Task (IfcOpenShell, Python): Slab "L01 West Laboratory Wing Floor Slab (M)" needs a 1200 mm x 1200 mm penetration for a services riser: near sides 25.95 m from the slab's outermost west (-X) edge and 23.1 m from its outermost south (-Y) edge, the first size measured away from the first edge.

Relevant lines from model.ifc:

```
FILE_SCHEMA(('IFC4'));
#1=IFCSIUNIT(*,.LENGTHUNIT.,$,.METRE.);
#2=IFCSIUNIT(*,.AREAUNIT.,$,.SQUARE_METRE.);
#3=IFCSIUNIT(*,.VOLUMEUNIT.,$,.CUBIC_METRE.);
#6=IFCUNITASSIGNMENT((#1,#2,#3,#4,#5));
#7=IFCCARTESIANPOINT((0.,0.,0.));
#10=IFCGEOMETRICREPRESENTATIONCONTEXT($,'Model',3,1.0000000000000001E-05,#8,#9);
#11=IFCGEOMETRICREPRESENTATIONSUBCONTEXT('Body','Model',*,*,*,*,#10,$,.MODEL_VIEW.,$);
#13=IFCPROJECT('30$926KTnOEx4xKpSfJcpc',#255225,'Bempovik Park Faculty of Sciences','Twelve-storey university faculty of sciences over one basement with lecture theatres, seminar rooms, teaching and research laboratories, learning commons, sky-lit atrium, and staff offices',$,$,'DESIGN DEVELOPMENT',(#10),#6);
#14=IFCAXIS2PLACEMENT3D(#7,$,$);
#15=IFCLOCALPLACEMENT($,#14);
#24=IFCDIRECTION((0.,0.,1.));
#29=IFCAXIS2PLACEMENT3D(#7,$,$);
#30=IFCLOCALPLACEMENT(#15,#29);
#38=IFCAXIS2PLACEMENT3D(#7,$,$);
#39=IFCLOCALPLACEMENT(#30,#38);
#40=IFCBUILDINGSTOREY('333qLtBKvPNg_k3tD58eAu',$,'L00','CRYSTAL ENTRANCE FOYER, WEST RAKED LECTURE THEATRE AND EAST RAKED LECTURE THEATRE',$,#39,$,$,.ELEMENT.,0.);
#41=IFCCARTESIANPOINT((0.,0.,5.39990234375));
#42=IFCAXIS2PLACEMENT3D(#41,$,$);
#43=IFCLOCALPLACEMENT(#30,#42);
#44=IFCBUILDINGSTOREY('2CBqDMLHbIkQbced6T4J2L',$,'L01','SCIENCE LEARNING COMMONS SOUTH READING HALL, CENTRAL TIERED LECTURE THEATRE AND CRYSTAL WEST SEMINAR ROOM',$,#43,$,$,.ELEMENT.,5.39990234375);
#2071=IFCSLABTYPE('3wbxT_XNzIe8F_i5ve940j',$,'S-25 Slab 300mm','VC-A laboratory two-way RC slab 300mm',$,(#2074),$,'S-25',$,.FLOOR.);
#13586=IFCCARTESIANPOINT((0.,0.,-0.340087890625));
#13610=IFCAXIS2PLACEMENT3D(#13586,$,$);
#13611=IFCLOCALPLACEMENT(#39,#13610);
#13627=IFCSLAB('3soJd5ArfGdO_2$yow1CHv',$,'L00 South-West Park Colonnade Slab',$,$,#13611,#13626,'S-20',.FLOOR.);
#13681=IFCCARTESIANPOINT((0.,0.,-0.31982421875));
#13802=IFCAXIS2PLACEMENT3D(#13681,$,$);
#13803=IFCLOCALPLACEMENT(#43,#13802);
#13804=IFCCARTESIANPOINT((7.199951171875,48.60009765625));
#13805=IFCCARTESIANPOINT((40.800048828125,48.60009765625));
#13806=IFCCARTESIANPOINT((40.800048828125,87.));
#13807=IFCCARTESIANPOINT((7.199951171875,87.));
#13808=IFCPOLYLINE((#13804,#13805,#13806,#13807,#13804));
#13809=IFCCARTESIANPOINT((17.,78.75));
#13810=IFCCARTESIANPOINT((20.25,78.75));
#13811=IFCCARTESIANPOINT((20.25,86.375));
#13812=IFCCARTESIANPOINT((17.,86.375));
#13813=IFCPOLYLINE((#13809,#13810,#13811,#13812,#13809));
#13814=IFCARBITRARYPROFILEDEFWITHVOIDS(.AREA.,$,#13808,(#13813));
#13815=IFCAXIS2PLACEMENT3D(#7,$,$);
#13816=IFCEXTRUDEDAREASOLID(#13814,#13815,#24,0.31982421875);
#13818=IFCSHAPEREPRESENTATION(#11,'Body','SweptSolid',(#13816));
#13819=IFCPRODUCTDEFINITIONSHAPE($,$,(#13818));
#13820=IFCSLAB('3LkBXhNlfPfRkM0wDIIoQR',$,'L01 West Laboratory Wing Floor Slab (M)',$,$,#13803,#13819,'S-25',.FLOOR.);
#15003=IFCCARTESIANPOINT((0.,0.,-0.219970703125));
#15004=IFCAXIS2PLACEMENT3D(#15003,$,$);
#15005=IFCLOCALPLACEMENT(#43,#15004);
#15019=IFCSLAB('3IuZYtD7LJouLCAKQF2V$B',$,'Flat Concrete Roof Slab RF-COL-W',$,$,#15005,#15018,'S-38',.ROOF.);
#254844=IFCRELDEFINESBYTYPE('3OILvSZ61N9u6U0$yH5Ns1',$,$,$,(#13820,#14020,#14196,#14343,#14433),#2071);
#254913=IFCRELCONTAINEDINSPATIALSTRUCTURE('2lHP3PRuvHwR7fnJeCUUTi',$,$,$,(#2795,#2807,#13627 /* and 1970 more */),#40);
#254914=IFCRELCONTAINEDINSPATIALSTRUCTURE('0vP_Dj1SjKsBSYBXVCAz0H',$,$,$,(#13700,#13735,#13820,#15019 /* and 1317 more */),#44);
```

```python
import numpy as np
import ifcopenshell
import ifcopenshell.api.feature
import ifcopenshell.api.geometry
import ifcopenshell.api.root
import ifcopenshell.geom
import ifcopenshell.util.placement
import ifcopenshell.util.representation
import ifcopenshell.util.shape
import ifcopenshell.util.unit

model = ifcopenshell.open("model.ifc")
unit_scale = ifcopenshell.util.unit.calculate_unit_scale(model)
settings = ifcopenshell.geom.settings()


def volume(element):
    """Net volume in cubic metres, openings subtracted."""
    shape = ifcopenshell.geom.create_shape(settings, element)
    return ifcopenshell.util.shape.get_volume(shape.geometry)


slab = model.by_guid("3LkBXhNlfPfRkM0wDIIoQR")
before = volume(slab)

# Extent in the slab's own axes, in metres. The edges named are its -X and -Y sides.
slab_shape = ifcopenshell.geom.create_shape(settings, slab)
vertices = ifcopenshell.util.shape.get_vertices(slab_shape.geometry)
x_min, y_min, bottom = vertices.min(axis=0)
top = vertices[:, 2].max()

opening = ifcopenshell.api.root.create_entity(model, ifc_class="IfcOpeningElement", name="Services riser opening", predefined_type="OPENING")
context = ifcopenshell.util.representation.get_context(model, "Model", "Body", "MODEL_VIEW")
width, depth = 1.2, 1.2
outline = [(0.0, 0.0), (width, 0.0), (width, depth), (0.0, depth), (0.0, 0.0)]
# Overshoot both faces by 50 mm so the cut is clean.
shape = ifcopenshell.api.geometry.add_slab_representation(
    model, context=context, depth=top - bottom + 0.1, polyline=outline
)
ifcopenshell.api.geometry.assign_representation(model, product=opening, representation=shape)

matrix = ifcopenshell.util.placement.get_local_placement(slab.ObjectPlacement)
matrix[:, 3] = matrix @ np.append(np.array([x_min + 25.95, y_min + 23.1, bottom - 0.05]) / unit_scale, 1.0)
ifcopenshell.api.geometry.edit_object_placement(model, product=opening, matrix=matrix, is_si=False)
ifcopenshell.api.feature.add_feature(model, feature=opening, element=slab)

after = volume(slab)

print(f"slab volume {before:.3f} -> {after:.3f} m3")

model.write("model_updated.ifc")
```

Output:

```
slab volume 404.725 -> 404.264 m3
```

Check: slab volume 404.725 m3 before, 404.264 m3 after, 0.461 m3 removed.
